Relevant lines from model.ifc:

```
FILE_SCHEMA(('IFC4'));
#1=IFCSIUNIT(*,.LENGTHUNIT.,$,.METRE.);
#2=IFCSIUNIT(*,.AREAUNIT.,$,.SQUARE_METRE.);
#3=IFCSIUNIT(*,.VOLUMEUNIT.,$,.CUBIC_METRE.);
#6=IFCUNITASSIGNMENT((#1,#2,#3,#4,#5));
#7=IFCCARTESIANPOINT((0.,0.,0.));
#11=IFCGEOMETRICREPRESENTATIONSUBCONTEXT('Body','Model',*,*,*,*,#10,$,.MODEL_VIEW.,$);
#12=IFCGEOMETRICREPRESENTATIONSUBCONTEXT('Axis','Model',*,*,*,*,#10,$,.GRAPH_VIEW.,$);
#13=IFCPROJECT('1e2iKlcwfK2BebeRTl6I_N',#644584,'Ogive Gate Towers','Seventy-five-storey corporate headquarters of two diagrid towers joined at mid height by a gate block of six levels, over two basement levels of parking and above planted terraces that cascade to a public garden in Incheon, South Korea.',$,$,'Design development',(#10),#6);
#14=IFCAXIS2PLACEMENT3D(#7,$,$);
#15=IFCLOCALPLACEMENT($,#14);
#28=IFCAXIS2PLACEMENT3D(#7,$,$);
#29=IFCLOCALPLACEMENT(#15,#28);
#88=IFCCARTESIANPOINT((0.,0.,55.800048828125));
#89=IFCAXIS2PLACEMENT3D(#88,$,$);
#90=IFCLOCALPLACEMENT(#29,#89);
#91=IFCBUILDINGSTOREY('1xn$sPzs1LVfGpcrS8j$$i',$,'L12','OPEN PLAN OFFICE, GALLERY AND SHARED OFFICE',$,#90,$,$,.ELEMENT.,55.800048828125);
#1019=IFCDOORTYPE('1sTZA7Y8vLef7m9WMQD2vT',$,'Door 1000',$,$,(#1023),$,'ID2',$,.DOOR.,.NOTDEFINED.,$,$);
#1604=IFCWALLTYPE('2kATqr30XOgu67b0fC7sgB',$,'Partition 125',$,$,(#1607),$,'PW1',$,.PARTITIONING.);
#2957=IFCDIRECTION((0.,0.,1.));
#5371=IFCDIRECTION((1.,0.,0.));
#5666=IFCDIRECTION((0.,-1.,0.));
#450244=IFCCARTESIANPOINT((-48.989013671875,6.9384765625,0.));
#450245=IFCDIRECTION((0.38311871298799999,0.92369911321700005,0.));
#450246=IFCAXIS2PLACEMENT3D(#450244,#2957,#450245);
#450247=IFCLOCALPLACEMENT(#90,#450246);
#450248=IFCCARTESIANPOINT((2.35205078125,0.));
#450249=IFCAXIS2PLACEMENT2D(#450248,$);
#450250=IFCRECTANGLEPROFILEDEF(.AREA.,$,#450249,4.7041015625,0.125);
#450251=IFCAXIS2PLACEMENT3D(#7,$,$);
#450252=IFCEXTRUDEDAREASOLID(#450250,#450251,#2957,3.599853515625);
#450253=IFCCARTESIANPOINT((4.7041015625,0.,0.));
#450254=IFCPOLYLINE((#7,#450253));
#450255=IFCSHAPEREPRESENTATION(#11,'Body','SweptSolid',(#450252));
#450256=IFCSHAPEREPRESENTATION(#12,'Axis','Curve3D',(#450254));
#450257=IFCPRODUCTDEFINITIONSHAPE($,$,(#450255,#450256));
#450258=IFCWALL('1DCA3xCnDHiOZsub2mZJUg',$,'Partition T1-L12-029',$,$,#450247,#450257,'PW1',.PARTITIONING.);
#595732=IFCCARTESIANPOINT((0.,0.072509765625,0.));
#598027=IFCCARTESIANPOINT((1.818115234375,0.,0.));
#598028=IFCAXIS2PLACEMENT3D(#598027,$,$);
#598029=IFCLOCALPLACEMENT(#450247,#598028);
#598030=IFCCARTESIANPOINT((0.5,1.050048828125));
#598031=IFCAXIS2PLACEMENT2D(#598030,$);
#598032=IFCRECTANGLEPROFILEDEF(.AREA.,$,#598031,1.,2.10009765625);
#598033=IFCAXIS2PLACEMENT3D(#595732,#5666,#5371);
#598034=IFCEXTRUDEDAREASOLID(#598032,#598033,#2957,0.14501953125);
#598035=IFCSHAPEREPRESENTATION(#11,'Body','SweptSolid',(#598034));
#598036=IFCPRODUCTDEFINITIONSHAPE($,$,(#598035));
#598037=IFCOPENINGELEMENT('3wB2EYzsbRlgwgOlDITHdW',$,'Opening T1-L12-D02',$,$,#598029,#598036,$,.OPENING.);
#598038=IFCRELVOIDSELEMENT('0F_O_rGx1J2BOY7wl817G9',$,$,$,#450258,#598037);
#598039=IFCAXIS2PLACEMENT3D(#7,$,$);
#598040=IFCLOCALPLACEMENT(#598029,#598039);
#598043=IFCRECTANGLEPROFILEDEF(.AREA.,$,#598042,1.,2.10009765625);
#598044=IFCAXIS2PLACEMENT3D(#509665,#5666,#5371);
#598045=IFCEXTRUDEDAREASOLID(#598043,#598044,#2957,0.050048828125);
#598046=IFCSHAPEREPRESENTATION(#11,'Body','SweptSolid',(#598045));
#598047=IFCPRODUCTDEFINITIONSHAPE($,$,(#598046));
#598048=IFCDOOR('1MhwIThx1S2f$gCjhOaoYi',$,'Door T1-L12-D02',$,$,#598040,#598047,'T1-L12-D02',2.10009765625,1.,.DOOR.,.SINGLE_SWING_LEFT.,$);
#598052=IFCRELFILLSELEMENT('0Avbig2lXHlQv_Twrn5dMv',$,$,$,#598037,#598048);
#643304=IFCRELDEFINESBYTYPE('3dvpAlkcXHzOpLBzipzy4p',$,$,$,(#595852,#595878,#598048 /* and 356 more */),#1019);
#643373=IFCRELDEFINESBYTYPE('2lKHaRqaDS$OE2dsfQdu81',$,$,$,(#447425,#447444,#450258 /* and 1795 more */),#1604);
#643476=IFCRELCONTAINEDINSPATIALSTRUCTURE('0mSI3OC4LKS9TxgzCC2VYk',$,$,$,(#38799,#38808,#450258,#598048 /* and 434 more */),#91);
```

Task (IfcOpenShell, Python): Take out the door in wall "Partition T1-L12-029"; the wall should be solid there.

```python
import ifcopenshell
import ifcopenshell.api.feature
import ifcopenshell.api.root
import ifcopenshell.geom
import ifcopenshell.util.shape

model = ifcopenshell.open("model.ifc")
settings = ifcopenshell.geom.settings()


def volume(element):
    """Net volume in cubic metres, openings subtracted."""
    shape = ifcopenshell.geom.create_shape(settings, element)
    return ifcopenshell.util.shape.get_volume(shape.geometry)


door = model.by_guid("1MhwIThx1S2f$gCjhOaoYi")
opening = door.FillsVoids[0].RelatingOpeningElement
wall = opening.VoidsElements[0].RelatingBuildingElement
before = volume(wall)

ifcopenshell.api.root.remove_product(model, product=door)
ifcopenshell.api.feature.remove_feature(model, feature=opening)

after = volume(wall)

print(f"wall volume {before:.3f} -> {after:.3f} m3")

model.write("model_edited.ifc")
```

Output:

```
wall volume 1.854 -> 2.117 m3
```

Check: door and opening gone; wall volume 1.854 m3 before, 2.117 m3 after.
